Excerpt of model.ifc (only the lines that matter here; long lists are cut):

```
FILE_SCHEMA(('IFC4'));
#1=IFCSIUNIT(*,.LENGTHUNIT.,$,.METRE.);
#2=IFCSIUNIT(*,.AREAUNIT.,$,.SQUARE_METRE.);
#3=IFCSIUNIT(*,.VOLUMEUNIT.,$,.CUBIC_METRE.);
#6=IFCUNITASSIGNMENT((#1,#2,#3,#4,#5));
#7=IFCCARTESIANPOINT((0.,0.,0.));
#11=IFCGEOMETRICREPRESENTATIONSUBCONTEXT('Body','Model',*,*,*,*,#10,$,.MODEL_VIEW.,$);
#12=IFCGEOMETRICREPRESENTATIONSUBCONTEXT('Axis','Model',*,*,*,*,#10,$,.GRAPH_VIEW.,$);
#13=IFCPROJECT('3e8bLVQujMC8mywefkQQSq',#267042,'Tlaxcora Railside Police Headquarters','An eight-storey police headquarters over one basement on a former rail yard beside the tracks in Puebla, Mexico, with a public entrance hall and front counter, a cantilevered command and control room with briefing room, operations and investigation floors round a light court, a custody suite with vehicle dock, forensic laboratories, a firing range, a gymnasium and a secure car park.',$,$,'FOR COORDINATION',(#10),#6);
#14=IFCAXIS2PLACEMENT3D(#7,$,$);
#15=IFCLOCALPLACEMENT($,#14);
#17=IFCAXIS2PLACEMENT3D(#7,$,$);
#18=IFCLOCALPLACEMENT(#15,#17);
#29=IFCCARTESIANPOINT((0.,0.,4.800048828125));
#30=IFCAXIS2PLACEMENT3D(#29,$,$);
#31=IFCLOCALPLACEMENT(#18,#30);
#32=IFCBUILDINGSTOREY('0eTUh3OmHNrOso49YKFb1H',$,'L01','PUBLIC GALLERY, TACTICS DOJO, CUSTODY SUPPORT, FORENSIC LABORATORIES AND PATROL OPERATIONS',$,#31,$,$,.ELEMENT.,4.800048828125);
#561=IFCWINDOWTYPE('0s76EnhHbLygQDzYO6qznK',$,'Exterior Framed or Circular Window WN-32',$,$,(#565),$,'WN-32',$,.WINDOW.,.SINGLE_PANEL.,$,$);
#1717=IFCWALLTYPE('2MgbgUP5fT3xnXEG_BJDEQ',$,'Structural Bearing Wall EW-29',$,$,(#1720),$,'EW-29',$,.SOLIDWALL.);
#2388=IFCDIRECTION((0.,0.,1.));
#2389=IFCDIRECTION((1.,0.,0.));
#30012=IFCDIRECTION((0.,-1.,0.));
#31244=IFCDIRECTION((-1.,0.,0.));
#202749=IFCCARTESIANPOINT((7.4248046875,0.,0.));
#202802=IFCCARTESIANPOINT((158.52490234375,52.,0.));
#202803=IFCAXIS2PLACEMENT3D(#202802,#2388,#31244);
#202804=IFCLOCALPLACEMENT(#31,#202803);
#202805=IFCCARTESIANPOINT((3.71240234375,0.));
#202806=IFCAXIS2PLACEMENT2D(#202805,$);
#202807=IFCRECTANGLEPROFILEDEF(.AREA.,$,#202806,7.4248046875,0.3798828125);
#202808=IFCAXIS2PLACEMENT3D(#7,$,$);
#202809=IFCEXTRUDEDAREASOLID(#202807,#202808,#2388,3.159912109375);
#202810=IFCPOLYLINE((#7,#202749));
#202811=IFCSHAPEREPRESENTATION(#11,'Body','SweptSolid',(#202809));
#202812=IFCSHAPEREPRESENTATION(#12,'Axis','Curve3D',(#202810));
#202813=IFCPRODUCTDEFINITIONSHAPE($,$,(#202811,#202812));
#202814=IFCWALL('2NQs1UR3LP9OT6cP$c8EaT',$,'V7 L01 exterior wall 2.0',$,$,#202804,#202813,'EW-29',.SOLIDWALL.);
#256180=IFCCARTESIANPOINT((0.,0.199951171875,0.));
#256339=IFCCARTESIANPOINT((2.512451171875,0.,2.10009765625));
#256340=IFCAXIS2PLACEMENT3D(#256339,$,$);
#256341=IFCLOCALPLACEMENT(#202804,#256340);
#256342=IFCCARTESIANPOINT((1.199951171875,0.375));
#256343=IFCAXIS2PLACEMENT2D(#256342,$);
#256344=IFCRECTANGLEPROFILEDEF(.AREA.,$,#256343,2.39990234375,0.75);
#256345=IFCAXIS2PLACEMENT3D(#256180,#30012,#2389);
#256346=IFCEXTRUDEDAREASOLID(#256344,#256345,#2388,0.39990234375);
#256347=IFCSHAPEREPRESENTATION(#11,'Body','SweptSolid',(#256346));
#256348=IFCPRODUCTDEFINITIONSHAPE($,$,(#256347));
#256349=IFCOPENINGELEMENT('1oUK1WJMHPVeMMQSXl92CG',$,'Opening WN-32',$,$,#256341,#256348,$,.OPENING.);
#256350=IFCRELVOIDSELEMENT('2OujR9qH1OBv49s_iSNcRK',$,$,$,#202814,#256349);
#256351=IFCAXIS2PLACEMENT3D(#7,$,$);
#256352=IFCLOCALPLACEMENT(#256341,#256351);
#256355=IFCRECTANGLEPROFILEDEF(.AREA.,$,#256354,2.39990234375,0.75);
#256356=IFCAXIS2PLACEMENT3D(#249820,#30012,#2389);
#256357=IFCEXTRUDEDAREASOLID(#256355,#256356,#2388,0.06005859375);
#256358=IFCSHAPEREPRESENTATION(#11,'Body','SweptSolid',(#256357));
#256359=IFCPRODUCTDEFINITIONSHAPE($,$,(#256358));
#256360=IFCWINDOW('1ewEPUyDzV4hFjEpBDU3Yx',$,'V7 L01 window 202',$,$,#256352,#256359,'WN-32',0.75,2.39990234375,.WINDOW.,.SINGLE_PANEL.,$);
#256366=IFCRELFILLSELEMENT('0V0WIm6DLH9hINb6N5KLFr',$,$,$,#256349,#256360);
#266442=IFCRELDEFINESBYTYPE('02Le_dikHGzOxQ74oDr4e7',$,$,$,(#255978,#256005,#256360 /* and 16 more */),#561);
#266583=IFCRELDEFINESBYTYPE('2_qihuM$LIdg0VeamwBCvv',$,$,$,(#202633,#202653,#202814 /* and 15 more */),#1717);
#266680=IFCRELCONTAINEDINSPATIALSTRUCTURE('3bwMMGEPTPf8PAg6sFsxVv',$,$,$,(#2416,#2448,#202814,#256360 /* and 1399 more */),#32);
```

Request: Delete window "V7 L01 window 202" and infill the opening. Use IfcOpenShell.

```python
import ifcopenshell
import ifcopenshell.api.feature
import ifcopenshell.api.root
import ifcopenshell.geom
import ifcopenshell.util.shape

model = ifcopenshell.open("model.ifc")
settings = ifcopenshell.geom.settings()


def volume(element):
    """Net volume in cubic metres, openings subtracted."""
    shape = ifcopenshell.geom.create_shape(settings, element)
    return ifcopenshell.util.shape.get_volume(shape.geometry)


window = model.by_guid("1ewEPUyDzV4hFjEpBDU3Yx")
opening = window.FillsVoids[0].RelatingOpeningElement
wall = opening.VoidsElements[0].RelatingBuildingElement
before = volume(wall)

ifcopenshell.api.root.remove_product(model, product=window)
ifcopenshell.api.feature.remove_feature(model, feature=opening)

after = volume(wall)

print(f"wall volume {before:.3f} -> {after:.3f} m3")

model.write("model_v2.ifc")
```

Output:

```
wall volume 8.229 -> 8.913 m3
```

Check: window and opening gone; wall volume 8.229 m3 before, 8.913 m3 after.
